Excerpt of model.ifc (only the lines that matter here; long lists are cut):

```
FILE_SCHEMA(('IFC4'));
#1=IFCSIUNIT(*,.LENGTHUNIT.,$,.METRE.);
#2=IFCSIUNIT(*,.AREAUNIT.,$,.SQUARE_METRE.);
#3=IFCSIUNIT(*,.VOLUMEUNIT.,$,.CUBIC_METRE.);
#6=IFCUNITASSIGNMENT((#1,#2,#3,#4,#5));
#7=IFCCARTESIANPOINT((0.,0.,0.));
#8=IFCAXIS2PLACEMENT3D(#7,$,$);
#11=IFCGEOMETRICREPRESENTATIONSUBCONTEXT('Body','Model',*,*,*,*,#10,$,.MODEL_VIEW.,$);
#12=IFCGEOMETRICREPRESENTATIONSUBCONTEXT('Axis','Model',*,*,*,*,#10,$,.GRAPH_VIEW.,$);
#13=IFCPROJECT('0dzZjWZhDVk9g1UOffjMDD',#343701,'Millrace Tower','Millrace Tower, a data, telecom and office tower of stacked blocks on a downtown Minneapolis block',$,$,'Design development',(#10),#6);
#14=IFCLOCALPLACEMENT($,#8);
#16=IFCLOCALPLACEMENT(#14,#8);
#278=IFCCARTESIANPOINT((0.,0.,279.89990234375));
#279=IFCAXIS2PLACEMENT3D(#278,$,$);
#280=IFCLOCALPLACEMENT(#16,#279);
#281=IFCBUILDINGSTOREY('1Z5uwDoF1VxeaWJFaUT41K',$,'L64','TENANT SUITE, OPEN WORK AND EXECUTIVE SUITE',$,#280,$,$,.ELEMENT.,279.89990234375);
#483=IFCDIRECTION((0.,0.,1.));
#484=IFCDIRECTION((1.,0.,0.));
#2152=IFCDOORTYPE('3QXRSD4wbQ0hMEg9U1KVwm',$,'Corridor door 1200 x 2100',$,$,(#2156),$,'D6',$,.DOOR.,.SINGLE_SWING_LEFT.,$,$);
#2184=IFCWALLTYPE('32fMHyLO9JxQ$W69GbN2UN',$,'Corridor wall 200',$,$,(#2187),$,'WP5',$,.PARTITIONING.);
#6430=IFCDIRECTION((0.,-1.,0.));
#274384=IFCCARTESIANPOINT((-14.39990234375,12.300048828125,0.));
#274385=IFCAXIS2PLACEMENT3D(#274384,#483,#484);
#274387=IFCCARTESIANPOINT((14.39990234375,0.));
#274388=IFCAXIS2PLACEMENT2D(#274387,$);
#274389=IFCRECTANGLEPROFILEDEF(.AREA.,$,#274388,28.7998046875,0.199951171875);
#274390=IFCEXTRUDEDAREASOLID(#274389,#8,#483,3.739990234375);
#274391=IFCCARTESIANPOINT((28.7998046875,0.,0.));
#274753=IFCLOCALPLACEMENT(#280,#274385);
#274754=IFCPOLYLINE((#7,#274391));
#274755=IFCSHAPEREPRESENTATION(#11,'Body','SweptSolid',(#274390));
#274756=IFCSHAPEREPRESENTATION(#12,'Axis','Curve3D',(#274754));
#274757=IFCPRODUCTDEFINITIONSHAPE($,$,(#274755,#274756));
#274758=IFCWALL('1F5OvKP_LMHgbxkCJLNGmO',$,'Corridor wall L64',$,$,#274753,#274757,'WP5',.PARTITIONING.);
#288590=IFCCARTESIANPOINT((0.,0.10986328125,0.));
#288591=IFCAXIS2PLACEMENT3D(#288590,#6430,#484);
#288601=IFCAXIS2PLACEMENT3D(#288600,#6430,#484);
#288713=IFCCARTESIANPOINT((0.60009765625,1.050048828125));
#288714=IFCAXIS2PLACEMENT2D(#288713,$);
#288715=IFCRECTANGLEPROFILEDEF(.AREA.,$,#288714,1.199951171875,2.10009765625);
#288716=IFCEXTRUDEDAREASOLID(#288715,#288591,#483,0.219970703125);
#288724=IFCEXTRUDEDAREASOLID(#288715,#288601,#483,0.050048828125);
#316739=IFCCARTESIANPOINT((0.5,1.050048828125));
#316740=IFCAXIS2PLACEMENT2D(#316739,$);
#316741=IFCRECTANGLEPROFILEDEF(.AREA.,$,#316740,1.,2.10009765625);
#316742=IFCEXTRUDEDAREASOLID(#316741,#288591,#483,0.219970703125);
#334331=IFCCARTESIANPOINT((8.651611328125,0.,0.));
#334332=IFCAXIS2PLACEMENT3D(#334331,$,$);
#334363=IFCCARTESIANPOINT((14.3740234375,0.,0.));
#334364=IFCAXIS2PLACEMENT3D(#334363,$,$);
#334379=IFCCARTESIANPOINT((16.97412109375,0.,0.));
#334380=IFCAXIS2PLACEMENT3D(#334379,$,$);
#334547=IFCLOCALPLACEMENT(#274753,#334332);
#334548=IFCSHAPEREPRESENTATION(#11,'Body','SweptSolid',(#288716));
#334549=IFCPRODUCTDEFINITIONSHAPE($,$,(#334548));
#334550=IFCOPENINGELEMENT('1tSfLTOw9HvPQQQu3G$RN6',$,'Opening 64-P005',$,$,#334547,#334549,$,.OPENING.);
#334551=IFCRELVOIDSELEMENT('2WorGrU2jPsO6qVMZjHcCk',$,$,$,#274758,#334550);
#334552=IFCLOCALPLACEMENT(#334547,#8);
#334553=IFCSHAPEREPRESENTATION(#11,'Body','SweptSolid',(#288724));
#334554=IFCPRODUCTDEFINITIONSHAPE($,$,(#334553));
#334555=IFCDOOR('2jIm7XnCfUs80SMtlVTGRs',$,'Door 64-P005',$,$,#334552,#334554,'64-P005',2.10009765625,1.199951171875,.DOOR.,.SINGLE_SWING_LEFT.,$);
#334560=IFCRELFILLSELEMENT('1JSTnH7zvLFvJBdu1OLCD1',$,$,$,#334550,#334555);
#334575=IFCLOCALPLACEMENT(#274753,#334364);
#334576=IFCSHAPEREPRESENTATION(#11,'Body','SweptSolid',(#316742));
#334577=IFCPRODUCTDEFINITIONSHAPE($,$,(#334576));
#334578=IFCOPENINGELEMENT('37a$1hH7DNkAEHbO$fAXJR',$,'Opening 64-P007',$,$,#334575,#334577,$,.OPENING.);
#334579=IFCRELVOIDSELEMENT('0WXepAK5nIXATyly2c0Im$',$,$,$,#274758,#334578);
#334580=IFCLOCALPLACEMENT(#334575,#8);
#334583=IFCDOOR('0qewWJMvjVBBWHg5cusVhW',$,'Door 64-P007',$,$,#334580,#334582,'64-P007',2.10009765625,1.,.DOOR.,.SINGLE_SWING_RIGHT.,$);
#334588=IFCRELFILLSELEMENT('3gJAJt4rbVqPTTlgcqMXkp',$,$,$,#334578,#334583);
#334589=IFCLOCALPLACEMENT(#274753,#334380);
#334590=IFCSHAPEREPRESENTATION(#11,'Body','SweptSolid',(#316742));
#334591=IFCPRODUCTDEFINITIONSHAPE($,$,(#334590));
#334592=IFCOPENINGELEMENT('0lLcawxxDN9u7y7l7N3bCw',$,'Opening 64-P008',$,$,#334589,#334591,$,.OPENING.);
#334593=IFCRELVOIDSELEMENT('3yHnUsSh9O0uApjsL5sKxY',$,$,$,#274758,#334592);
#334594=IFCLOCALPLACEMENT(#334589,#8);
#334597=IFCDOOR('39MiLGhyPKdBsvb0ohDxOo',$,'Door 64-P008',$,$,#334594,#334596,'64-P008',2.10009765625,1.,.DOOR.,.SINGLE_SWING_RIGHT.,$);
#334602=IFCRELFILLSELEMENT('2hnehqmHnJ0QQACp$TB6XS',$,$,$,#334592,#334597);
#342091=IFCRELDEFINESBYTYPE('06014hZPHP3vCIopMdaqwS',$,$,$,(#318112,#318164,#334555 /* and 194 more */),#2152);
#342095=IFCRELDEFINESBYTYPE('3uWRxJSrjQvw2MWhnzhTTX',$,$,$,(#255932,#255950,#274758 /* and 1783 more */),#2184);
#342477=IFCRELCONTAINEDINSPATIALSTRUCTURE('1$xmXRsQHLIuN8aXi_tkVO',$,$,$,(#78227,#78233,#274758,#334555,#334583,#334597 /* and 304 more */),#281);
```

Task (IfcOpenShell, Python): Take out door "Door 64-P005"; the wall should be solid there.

```python
import ifcopenshell
import ifcopenshell.api.feature
import ifcopenshell.api.root
import ifcopenshell.geom
import ifcopenshell.util.shape

model = ifcopenshell.open("model.ifc")
settings = ifcopenshell.geom.settings()


def volume(element):
    """Net volume in cubic metres, openings subtracted."""
    shape = ifcopenshell.geom.create_shape(settings, element)
    return ifcopenshell.util.shape.get_volume(shape.geometry)


door = model.by_guid("2jIm7XnCfUs80SMtlVTGRs")
opening = door.FillsVoids[0].RelatingOpeningElement
wall = opening.VoidsElements[0].RelatingBuildingElement
before = volume(wall)

ifcopenshell.api.root.remove_product(model, product=door)
ifcopenshell.api.feature.remove_feature(model, feature=opening)

after = volume(wall)

print(f"wall volume {before:.3f} -> {after:.3f} m3")

model.write("model_rev.ifc")
```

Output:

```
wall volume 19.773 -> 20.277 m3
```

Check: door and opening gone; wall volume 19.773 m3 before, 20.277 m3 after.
